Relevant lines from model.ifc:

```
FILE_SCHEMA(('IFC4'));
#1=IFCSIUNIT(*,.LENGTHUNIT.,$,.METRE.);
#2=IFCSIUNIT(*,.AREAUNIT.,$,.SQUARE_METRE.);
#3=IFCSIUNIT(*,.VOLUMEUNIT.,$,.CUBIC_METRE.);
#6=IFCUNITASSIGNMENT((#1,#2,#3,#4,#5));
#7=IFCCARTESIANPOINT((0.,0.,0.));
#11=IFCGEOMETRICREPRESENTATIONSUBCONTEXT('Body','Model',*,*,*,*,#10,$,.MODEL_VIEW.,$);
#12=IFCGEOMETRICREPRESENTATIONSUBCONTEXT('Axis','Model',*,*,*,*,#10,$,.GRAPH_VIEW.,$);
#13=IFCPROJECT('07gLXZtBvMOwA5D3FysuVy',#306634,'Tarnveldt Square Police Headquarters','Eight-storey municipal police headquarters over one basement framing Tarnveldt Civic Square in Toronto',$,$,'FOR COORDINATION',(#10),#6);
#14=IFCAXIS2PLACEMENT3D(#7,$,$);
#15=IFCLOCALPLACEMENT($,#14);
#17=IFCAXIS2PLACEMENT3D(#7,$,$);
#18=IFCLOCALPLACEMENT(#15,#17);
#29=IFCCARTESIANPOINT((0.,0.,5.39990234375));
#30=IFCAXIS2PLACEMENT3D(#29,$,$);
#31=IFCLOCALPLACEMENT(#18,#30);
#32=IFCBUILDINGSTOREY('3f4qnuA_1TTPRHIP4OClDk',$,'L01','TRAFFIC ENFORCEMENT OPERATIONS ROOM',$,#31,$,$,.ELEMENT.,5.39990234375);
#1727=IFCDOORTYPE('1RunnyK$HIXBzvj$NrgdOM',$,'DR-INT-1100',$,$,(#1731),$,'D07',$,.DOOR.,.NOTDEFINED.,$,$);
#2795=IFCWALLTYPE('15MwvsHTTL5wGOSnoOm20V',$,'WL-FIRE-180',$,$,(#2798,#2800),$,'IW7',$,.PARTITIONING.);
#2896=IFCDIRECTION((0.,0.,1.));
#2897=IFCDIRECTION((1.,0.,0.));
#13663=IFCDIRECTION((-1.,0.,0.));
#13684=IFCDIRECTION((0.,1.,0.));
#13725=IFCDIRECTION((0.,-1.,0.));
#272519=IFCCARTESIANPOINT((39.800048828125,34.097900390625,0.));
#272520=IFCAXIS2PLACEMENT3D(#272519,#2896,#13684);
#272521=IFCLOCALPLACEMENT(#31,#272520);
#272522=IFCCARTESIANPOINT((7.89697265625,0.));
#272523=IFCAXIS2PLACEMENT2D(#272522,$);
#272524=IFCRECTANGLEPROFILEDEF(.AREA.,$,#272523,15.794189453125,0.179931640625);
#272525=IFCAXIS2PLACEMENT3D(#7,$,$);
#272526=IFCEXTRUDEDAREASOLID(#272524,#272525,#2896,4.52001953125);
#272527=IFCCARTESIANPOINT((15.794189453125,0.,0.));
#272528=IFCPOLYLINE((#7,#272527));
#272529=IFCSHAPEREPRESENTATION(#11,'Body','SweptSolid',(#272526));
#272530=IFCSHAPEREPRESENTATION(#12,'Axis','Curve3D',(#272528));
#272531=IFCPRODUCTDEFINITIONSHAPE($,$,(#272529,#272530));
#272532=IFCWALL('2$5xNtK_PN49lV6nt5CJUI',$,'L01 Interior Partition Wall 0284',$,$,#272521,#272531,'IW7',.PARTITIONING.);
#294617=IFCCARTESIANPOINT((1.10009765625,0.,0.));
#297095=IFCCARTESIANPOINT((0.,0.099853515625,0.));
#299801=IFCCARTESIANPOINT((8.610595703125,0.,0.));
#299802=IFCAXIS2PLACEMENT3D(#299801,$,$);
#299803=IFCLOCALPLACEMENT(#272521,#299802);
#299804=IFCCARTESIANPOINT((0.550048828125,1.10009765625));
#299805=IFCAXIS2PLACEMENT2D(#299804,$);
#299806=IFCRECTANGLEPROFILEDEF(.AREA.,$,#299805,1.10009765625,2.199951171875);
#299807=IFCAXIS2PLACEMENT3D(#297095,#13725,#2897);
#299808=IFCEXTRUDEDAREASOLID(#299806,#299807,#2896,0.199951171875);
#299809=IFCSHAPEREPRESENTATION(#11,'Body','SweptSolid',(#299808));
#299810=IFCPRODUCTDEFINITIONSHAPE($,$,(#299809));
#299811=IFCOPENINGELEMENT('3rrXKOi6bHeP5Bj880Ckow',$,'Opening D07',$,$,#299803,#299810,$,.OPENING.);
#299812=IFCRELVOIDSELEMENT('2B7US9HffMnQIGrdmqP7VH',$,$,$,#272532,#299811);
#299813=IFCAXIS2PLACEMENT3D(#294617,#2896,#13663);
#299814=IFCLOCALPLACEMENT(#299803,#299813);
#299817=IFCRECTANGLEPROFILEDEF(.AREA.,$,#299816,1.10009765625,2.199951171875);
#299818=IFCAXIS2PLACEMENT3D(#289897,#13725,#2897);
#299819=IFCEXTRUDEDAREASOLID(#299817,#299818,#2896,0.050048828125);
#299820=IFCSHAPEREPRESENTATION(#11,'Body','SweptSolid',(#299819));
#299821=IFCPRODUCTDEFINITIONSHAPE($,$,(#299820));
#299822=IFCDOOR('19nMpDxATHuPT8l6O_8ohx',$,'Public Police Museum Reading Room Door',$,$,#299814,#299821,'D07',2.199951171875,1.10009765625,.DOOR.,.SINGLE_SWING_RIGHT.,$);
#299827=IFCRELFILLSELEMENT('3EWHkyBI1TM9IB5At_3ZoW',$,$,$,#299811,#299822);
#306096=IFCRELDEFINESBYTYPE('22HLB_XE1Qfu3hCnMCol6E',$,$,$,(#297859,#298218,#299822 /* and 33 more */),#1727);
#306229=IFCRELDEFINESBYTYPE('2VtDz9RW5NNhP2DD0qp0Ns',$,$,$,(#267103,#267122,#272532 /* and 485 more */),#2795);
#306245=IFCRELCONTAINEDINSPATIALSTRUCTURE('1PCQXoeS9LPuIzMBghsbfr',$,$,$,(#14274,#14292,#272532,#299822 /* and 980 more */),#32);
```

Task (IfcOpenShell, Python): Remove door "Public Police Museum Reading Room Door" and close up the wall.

```python
import ifcopenshell
import ifcopenshell.api.feature
import ifcopenshell.api.root
import ifcopenshell.geom
import ifcopenshell.util.shape

model = ifcopenshell.open("model.ifc")
settings = ifcopenshell.geom.settings()


def volume(element):
    """Net volume in cubic metres, openings subtracted."""
    shape = ifcopenshell.geom.create_shape(settings, element)
    return ifcopenshell.util.shape.get_volume(shape.geometry)


door = model.by_guid("19nMpDxATHuPT8l6O_8ohx")
opening = door.FillsVoids[0].RelatingOpeningElement
wall = opening.VoidsElements[0].RelatingBuildingElement
before = volume(wall)

ifcopenshell.api.root.remove_product(model, product=door)
ifcopenshell.api.feature.remove_feature(model, feature=opening)

after = volume(wall)

print(f"wall volume {before:.3f} -> {after:.3f} m3")

model.write("model_v2.ifc")
```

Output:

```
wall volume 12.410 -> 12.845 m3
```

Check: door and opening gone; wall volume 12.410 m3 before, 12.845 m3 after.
